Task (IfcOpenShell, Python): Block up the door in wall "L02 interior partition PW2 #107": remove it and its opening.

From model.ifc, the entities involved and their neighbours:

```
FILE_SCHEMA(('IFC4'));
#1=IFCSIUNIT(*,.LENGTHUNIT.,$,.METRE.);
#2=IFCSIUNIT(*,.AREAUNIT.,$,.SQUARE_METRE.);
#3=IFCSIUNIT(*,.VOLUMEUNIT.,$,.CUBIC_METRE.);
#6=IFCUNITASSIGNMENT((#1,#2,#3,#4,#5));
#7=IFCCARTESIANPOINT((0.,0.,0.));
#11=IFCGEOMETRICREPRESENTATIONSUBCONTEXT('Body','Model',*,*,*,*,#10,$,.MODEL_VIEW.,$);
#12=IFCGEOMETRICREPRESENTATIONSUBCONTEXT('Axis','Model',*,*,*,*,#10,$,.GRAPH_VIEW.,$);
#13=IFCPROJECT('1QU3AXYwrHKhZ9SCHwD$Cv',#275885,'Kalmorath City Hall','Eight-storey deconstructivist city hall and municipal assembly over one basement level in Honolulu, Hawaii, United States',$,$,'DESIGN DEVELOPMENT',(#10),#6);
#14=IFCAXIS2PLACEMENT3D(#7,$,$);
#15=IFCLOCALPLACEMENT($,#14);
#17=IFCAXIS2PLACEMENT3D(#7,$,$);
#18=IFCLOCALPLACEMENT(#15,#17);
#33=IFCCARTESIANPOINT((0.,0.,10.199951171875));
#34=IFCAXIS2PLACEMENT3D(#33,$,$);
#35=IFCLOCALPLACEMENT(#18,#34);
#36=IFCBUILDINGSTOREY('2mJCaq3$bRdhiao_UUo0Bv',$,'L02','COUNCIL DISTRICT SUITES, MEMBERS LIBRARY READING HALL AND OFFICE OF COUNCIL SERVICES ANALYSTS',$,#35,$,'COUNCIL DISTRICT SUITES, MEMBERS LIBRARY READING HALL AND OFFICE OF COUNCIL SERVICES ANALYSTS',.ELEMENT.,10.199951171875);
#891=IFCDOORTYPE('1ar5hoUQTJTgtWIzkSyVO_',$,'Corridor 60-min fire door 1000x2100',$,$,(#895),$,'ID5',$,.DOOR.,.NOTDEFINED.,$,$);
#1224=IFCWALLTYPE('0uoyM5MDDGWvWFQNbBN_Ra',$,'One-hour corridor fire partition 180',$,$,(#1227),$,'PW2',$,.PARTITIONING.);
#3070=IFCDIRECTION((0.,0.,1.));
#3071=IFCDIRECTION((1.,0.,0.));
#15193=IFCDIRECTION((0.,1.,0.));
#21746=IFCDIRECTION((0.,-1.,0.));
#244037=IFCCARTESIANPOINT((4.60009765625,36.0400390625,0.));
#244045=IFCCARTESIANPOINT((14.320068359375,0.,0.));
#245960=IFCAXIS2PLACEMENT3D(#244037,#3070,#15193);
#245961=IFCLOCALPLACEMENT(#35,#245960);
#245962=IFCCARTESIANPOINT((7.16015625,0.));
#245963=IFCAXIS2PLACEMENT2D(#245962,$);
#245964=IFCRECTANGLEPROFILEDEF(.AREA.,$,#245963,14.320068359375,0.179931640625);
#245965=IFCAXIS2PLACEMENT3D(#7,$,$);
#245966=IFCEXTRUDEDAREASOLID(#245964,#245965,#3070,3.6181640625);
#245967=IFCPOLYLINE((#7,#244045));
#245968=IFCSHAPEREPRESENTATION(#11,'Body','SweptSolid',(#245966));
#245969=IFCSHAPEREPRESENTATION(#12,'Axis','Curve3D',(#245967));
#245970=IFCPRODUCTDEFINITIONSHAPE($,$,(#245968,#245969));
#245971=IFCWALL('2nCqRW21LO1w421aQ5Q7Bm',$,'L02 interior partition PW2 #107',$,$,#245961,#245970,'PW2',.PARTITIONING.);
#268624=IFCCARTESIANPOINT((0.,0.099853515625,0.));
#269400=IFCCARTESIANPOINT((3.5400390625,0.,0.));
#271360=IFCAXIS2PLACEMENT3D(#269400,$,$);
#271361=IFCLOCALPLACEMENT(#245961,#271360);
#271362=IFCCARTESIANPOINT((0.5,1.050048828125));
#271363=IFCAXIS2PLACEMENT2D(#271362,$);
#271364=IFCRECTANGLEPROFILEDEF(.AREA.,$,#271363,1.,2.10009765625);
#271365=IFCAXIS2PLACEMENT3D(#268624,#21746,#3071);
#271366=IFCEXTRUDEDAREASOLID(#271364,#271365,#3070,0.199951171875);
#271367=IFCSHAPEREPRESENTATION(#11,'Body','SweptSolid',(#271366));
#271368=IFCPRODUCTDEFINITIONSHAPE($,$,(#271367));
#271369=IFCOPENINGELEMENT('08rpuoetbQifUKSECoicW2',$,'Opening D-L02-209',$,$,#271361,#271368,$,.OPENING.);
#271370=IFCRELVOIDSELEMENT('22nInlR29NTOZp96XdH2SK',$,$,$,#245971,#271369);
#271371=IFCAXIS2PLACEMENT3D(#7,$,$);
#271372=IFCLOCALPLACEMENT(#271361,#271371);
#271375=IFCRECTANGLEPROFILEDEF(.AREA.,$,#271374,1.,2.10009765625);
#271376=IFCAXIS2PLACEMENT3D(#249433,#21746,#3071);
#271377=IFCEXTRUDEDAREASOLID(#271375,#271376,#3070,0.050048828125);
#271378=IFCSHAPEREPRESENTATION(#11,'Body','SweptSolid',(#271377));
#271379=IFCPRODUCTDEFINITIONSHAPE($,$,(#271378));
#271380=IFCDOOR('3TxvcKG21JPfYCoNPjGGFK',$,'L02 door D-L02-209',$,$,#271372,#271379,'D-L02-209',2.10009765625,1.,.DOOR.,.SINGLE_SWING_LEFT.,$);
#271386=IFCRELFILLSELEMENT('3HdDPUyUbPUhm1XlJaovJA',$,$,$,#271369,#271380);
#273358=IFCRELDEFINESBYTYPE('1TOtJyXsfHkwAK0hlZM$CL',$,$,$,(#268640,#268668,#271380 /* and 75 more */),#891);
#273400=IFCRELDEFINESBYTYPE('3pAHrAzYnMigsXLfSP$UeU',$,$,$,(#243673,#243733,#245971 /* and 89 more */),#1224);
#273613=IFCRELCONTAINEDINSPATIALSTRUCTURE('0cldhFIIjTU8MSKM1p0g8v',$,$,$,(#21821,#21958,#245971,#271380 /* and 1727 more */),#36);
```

```python
import ifcopenshell
import ifcopenshell.api.feature
import ifcopenshell.api.root
import ifcopenshell.geom
import ifcopenshell.util.shape

model = ifcopenshell.open("model.ifc")
settings = ifcopenshell.geom.settings()


def volume(element):
    """Net volume in cubic metres, openings subtracted."""
    shape = ifcopenshell.geom.create_shape(settings, element)
    return ifcopenshell.util.shape.get_volume(shape.geometry)


door = model.by_id(271380)
opening = door.FillsVoids[0].RelatingOpeningElement
wall = opening.VoidsElements[0].RelatingBuildingElement
before = volume(wall)

ifcopenshell.api.root.remove_product(model, product=door)
ifcopenshell.api.feature.remove_feature(model, feature=opening)

after = volume(wall)

print(f"wall volume {before:.3f} -> {after:.3f} m3")

model.write("model_v2.ifc")
```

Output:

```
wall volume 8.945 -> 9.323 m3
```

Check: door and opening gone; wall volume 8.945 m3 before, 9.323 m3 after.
